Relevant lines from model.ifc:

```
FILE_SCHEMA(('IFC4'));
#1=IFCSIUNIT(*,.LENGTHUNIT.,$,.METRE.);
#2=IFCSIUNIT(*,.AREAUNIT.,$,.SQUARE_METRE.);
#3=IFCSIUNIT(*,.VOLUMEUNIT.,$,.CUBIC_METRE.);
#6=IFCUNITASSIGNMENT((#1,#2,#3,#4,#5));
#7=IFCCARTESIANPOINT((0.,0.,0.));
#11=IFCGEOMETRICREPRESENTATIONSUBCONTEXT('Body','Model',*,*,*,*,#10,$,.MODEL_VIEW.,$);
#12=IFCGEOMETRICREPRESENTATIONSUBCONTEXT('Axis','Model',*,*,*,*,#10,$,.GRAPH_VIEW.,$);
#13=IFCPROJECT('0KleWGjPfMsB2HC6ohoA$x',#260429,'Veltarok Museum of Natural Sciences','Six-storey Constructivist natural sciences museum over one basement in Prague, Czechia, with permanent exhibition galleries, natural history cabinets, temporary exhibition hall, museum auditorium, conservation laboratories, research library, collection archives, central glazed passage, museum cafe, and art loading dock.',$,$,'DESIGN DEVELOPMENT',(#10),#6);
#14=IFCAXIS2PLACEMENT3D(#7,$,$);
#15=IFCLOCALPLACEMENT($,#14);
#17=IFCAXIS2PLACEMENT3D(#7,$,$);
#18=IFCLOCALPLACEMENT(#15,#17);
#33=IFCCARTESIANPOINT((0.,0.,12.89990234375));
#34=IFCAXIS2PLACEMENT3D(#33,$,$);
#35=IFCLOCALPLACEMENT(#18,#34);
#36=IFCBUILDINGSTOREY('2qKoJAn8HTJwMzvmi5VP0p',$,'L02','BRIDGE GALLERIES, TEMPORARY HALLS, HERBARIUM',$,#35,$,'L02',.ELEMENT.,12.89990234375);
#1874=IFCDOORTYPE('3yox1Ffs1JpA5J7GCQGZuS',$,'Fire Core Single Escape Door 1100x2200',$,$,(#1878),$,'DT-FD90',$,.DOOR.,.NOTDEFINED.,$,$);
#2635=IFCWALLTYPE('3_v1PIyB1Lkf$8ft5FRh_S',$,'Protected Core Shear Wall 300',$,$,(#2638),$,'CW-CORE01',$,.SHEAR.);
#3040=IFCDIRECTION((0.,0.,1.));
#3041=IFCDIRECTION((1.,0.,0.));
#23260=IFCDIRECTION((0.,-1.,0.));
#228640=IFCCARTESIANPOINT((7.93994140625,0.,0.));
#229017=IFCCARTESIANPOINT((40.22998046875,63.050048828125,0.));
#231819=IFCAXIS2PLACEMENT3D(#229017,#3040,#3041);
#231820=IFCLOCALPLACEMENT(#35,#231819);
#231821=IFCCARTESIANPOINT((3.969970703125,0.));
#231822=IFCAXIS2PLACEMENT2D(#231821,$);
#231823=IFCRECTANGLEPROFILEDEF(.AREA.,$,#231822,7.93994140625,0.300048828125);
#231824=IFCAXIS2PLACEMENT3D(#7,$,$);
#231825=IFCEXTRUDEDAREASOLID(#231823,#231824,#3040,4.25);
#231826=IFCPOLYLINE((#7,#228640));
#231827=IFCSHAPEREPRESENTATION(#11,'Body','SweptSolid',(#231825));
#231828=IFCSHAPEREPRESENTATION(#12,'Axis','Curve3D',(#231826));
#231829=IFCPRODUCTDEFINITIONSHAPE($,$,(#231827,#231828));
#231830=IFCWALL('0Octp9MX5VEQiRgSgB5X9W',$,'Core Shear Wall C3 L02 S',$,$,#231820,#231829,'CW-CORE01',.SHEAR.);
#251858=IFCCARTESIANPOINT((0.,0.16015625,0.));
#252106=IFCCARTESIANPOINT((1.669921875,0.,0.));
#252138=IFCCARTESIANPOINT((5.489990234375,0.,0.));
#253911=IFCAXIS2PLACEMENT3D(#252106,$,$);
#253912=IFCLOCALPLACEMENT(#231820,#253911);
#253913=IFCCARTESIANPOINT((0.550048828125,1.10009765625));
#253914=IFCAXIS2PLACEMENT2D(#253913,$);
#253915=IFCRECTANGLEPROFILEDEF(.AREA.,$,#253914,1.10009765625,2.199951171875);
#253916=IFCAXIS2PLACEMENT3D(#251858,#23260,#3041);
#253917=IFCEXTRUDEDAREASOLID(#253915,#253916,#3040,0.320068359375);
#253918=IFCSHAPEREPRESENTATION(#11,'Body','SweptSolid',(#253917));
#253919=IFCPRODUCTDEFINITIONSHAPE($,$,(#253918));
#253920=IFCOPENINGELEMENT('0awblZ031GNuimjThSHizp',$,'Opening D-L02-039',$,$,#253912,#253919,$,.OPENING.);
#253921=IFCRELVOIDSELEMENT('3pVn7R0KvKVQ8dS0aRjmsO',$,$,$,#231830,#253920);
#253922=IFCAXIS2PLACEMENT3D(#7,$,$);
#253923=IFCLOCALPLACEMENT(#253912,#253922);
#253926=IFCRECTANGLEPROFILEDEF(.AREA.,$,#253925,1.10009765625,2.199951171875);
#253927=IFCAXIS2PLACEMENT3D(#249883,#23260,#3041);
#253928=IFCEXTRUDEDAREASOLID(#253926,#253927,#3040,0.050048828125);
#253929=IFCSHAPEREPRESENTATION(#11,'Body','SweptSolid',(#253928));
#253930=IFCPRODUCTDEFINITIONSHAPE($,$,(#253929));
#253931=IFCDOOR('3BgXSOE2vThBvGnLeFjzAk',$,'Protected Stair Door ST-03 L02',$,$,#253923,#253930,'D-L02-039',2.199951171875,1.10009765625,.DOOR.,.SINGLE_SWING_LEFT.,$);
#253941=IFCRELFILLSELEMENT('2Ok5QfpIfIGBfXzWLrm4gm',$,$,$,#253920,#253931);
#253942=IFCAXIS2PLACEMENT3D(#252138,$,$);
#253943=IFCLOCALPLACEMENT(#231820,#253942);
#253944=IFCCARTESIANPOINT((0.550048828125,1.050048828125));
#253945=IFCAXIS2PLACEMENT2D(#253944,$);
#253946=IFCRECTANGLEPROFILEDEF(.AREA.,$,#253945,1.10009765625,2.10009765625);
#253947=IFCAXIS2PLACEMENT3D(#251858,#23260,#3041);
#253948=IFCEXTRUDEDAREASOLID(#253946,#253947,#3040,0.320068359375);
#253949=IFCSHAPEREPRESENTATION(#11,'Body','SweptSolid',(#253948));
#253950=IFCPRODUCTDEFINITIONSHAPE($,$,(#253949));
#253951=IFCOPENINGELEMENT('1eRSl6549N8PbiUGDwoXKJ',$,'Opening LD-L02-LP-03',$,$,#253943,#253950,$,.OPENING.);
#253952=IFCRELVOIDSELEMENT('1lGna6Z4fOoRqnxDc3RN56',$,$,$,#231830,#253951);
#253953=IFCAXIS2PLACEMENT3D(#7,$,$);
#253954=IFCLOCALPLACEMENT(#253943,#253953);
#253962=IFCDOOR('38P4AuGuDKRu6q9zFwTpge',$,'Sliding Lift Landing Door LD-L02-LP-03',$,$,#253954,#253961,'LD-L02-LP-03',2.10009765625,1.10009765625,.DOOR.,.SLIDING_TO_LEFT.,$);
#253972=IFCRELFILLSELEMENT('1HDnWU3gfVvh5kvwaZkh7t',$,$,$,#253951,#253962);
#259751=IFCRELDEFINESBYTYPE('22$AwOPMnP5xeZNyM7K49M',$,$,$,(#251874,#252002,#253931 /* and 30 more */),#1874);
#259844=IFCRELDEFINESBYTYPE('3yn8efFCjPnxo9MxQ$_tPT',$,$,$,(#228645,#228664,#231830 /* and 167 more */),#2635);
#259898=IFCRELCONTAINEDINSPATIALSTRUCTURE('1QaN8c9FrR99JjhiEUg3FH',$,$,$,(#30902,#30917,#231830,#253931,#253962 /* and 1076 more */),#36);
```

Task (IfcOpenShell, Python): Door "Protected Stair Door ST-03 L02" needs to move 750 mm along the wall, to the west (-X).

```python
import ifcopenshell
import ifcopenshell.api.geometry
import ifcopenshell.util.placement

model = ifcopenshell.open("model.ifc")

door = model.by_guid("3BgXSOE2vThBvGnLeFjzAk")
opening = door.FillsVoids[0].RelatingOpeningElement
wall = opening.VoidsElements[0].RelatingBuildingElement

wall_matrix = ifcopenshell.util.placement.get_local_placement(wall.ObjectPlacement)
shift = wall_matrix[:3, 0] * -0.75
before = ifcopenshell.util.placement.get_local_placement(door.ObjectPlacement)[:3, 3].copy()

# The door is placed relative to its opening, so it follows when the opening moves.
matrix = ifcopenshell.util.placement.get_local_placement(opening.ObjectPlacement)
matrix[:3, 3] += shift
ifcopenshell.api.geometry.edit_object_placement(
    model, product=opening, matrix=matrix, is_si=False, should_transform_children=True
)

after = ifcopenshell.util.placement.get_local_placement(door.ObjectPlacement)[:3, 3]
print("door moved by", (after - before).round(3) + 0.0)

model.write("model-out.ifc")
```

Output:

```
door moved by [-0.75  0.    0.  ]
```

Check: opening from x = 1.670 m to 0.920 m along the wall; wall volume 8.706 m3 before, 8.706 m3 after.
